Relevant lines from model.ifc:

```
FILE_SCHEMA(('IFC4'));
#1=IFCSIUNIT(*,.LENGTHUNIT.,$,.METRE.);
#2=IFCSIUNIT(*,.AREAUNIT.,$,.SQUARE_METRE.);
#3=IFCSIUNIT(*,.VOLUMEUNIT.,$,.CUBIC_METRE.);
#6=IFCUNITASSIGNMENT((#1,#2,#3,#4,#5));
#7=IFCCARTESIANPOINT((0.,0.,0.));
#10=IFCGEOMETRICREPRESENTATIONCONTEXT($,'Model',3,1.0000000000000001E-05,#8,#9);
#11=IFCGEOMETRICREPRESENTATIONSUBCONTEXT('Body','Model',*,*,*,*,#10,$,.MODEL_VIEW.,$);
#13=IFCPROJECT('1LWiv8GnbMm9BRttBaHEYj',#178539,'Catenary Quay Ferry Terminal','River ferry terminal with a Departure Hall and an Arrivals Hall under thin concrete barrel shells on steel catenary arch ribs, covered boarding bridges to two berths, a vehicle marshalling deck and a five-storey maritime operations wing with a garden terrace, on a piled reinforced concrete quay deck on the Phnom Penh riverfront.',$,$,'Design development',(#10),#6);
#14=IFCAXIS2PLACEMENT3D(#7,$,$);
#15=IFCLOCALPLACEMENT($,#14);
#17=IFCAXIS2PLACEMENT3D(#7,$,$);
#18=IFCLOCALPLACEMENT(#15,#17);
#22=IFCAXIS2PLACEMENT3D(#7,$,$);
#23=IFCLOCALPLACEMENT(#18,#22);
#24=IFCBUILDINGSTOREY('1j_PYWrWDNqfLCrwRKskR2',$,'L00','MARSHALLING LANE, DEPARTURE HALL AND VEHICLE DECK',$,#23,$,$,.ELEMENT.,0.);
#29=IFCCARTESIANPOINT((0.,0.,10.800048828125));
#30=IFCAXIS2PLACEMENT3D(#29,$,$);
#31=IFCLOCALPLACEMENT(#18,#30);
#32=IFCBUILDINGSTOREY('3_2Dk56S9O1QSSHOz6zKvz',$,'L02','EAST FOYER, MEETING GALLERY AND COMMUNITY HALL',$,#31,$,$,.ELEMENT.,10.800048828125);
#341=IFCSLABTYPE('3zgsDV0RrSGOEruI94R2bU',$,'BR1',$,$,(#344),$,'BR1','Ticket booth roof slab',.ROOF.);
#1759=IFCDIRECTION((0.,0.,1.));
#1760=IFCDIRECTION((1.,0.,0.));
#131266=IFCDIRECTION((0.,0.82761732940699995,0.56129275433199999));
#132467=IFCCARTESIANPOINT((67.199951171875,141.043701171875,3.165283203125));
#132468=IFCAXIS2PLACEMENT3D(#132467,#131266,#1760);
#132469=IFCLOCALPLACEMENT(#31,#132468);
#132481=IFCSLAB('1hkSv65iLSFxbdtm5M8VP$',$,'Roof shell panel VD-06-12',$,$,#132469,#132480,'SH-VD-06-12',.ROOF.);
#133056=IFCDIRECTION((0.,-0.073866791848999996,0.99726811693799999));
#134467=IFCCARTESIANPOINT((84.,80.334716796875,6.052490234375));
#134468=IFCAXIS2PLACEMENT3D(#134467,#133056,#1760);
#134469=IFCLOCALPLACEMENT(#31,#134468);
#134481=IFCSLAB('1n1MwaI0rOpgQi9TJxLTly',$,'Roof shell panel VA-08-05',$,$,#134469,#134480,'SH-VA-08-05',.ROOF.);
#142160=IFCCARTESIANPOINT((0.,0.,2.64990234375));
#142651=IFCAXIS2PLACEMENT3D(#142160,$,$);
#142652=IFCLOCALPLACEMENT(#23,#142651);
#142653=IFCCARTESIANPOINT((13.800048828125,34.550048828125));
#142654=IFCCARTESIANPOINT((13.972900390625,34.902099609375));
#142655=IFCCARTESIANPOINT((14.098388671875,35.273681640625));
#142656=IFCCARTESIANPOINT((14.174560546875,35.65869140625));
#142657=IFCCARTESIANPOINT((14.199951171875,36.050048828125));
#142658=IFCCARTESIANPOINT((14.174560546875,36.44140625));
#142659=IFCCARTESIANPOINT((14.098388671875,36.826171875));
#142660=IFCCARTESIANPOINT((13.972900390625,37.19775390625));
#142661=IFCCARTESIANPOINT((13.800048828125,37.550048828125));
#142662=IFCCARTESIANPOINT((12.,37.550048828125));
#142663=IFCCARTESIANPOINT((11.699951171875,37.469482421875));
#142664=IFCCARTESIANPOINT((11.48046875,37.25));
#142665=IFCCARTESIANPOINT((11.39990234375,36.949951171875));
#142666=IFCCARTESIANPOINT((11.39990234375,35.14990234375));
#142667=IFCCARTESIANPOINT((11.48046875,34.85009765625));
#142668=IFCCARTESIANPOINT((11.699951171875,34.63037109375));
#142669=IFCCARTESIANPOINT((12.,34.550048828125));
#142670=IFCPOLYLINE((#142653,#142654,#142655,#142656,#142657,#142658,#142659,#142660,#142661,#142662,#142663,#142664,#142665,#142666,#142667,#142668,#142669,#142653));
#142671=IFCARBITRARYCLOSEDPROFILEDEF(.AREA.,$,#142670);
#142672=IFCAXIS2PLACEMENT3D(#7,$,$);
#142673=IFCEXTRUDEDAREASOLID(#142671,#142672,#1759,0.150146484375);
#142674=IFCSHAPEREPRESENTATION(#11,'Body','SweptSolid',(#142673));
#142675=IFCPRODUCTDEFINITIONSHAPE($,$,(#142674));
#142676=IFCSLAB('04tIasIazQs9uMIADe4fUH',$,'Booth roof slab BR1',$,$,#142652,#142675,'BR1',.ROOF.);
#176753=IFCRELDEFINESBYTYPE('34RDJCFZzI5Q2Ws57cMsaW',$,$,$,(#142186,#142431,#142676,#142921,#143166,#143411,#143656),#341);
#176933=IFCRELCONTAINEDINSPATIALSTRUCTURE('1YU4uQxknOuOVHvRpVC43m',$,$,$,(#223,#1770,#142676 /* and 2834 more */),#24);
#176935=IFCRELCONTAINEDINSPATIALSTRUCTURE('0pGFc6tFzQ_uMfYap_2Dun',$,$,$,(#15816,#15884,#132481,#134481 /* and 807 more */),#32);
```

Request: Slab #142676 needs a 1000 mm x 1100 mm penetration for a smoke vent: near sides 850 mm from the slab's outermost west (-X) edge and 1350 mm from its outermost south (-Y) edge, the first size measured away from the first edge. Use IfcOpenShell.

```python
import numpy as np
import ifcopenshell
import ifcopenshell.api.feature
import ifcopenshell.api.geometry
import ifcopenshell.api.root
import ifcopenshell.geom
import ifcopenshell.util.placement
import ifcopenshell.util.representation
import ifcopenshell.util.shape
import ifcopenshell.util.unit

model = ifcopenshell.open("model.ifc")
unit_scale = ifcopenshell.util.unit.calculate_unit_scale(model)
settings = ifcopenshell.geom.settings()


def volume(element):
    """Net volume in cubic metres, openings subtracted."""
    shape = ifcopenshell.geom.create_shape(settings, element)
    return ifcopenshell.util.shape.get_volume(shape.geometry)


slab = model.by_guid("04tIasIazQs9uMIADe4fUH")
before = volume(slab)

# Extent in the slab's own axes, in metres. The edges named are its -X and -Y sides.
slab_shape = ifcopenshell.geom.create_shape(settings, slab)
vertices = ifcopenshell.util.shape.get_vertices(slab_shape.geometry)
x_min, y_min, bottom = vertices.min(axis=0)
top = vertices[:, 2].max()

opening = ifcopenshell.api.root.create_entity(model, ifc_class="IfcOpeningElement", name="Smoke vent opening", predefined_type="OPENING")
context = ifcopenshell.util.representation.get_context(model, "Model", "Body", "MODEL_VIEW")
width, depth = 1, 1.1
outline = [(0.0, 0.0), (width, 0.0), (width, depth), (0.0, depth), (0.0, 0.0)]
# Overshoot both faces by 50 mm so the cut is clean.
shape = ifcopenshell.api.geometry.add_slab_representation(
    model, context=context, depth=top - bottom + 0.1, polyline=outline
)
ifcopenshell.api.geometry.assign_representation(model, product=opening, representation=shape)

matrix = ifcopenshell.util.placement.get_local_placement(slab.ObjectPlacement)
matrix[:, 3] = matrix @ np.append(np.array([x_min + 0.85, y_min + 1.35, bottom - 0.05]) / unit_scale, 1.0)
ifcopenshell.api.geometry.edit_object_placement(model, product=opening, matrix=matrix, is_si=False)
ifcopenshell.api.feature.add_feature(model, feature=opening, element=slab)

after = volume(slab)

print(f"slab volume {before:.3f} -> {after:.3f} m3")

model.write("model_rev.ifc")
```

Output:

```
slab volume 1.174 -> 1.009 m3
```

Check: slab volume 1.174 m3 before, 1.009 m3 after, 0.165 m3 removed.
